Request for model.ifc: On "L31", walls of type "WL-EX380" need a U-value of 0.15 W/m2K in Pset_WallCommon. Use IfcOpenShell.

First a look at what the model holds.

```python
import ifcopenshell
import ifcopenshell.util.element

model = ifcopenshell.open("model.ifc")
print(model.schema)
storey = next(s for s in model.by_type("IfcBuildingStorey") if s.Name == "L31")
walls = [e for e in ifcopenshell.util.element.get_decomposition(storey) if e.is_a("IfcWall")]
seen = {}
for e in walls:
    element_type = ifcopenshell.util.element.get_type(e)
    key = (element_type.Name if element_type != e and element_type else None, ifcopenshell.util.element.get_pset(e, "Pset_WallCommon", "ThermalTransmittance"))
    seen[key] = seen.get(key, 0) + 1
for (name, value), count in sorted(seen.items(), key=str):
    print(count, "x", name, "|", value)
```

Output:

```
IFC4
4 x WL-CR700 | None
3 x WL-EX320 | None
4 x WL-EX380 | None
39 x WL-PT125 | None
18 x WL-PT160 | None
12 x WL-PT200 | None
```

```python
import ifcopenshell
import ifcopenshell.api.pset
import ifcopenshell.util.element

model = ifcopenshell.open("model.ifc")

storey = next(s for s in model.by_type("IfcBuildingStorey") if s.Name == "L31")
walls = [e for e in ifcopenshell.util.element.get_decomposition(storey) if e.is_a("IfcWall")]

count = 0
for e in walls:
    element_type = ifcopenshell.util.element.get_type(e)
    if element_type in (None, e) or element_type.Name != "WL-EX380":
        continue
    # add_pset returns the element's existing set when there is one.
    pset = ifcopenshell.api.pset.add_pset(model, product=e, name="Pset_WallCommon")
    ifcopenshell.api.pset.edit_pset(model, pset=pset, properties={"ThermalTransmittance": 0.15})
    count += 1

print(count, "walls updated")

model.write("model_updated.ifc")
```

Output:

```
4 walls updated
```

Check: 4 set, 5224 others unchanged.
